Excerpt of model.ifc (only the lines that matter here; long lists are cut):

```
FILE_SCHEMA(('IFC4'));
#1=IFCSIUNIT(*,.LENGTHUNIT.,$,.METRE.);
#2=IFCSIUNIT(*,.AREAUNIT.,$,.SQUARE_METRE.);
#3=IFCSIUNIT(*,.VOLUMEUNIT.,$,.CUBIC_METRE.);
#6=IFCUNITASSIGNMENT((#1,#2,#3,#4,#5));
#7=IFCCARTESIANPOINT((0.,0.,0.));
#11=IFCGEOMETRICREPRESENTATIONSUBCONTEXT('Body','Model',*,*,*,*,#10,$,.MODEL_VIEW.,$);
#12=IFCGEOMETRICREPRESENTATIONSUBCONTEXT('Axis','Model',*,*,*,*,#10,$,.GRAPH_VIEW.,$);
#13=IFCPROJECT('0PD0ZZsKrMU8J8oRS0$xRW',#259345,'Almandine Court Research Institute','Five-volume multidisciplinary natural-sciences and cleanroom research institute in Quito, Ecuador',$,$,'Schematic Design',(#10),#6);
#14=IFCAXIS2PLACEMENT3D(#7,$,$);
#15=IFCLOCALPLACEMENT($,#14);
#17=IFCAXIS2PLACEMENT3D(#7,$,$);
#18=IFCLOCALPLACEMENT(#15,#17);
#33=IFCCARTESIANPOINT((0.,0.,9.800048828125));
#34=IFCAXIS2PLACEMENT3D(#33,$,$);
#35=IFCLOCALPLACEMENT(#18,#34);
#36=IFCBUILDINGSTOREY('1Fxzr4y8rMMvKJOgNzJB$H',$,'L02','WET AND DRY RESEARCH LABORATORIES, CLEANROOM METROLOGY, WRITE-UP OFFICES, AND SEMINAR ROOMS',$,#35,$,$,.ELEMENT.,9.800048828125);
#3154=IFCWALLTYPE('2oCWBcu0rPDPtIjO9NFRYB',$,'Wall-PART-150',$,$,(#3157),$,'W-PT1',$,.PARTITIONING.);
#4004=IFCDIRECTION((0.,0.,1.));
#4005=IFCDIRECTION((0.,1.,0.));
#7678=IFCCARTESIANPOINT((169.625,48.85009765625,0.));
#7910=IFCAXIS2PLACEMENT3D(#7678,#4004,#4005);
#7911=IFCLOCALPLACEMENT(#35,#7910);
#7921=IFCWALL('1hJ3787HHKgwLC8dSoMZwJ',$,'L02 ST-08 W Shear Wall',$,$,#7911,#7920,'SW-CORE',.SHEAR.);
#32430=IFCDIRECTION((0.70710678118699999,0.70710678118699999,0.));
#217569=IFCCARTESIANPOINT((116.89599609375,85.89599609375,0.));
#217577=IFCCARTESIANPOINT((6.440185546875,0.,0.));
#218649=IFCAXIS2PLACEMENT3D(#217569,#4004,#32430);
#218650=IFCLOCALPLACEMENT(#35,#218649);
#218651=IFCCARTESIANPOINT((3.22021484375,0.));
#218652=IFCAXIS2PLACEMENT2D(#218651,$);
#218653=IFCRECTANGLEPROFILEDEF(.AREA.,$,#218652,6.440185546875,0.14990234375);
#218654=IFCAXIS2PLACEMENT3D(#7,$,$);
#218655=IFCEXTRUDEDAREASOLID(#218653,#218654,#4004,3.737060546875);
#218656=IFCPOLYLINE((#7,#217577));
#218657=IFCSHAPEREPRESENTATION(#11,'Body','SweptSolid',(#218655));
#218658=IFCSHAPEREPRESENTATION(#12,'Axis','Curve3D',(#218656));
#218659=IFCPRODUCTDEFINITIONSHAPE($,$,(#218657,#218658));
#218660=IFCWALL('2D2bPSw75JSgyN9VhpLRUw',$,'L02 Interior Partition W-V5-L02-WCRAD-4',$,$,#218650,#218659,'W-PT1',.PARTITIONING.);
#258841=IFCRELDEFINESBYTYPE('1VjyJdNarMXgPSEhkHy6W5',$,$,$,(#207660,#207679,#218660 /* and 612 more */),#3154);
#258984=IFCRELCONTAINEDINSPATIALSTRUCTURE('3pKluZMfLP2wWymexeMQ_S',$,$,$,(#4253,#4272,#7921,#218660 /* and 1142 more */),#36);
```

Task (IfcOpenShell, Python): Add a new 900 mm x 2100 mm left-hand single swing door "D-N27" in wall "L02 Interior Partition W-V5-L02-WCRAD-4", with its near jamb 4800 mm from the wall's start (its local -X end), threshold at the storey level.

```python
import numpy as np
import ifcopenshell
import ifcopenshell.api.feature
import ifcopenshell.api.geometry
import ifcopenshell.api.root
import ifcopenshell.api.spatial
import ifcopenshell.geom
import ifcopenshell.util.element
import ifcopenshell.util.placement
import ifcopenshell.util.representation
import ifcopenshell.util.shape
import ifcopenshell.util.unit

model = ifcopenshell.open("model.ifc")
unit_scale = ifcopenshell.util.unit.calculate_unit_scale(model)
settings = ifcopenshell.geom.settings()


def volume(element):
    """Net volume in cubic metres, openings subtracted."""
    shape = ifcopenshell.geom.create_shape(settings, element)
    return ifcopenshell.util.shape.get_volume(shape.geometry)


wall = model.by_guid("2D2bPSw75JSgyN9VhpLRUw")
storey = ifcopenshell.util.element.get_container(wall, ifc_class="IfcBuildingStorey")
context = ifcopenshell.util.representation.get_context(model, "Model", "Body", "MODEL_VIEW")
before = volume(wall)

width, height, from_end, sill = 0.9, 2.1, 4.8, 0.0  # metres

# The wall runs along its own X axis, and the end named is its -X end.
wall_shape = ifcopenshell.geom.create_shape(settings, wall)
x, y, z = ifcopenshell.util.shape.get_vertices(wall_shape.geometry).T
start = x.min() + from_end
face, thickness = float(y.min()), float(y.max() - y.min())
wall_matrix = ifcopenshell.util.placement.get_local_placement(wall.ObjectPlacement)
level = ifcopenshell.util.placement.get_local_placement(storey.ObjectPlacement)[2, 3]


def in_wall(x, y):
    """Placement at x, y metres in the wall's axes, at sill height."""
    matrix = wall_matrix.copy()
    matrix[:, 3] = wall_matrix @ np.array([x / unit_scale, y / unit_scale, 0.0, 1.0])
    matrix[2, 3] = level + sill / unit_scale
    return matrix


# Opening: a box that overshoots both wall faces by 50 mm.
opening = ifcopenshell.api.root.create_entity(model, ifc_class="IfcOpeningElement", predefined_type="OPENING")
box = ifcopenshell.api.geometry.add_wall_representation(
    model, context=context, length=width, height=height, thickness=thickness + 0.1
)
ifcopenshell.api.geometry.assign_representation(model, product=opening, representation=box)
ifcopenshell.api.geometry.edit_object_placement(model, product=opening, matrix=in_wall(start, face - 0.05), is_si=False)
ifcopenshell.api.feature.add_feature(model, feature=opening, element=wall)

door = ifcopenshell.api.root.create_entity(model, ifc_class="IfcDoor", name="D-N27", predefined_type="DOOR")
door.OverallWidth, door.OverallHeight = width / unit_scale, height / unit_scale
door.OperationType = "SINGLE_SWING_LEFT"
body = ifcopenshell.api.geometry.add_door_representation(
    model,
    context=context,
    overall_width=door.OverallWidth,
    overall_height=door.OverallHeight,
    operation_type="SINGLE_SWING_LEFT",
    lining_properties={"LiningDepth": thickness / unit_scale, "ThresholdDepth": thickness / unit_scale},
)
ifcopenshell.api.geometry.assign_representation(model, product=door, representation=body)
ifcopenshell.api.spatial.assign_container(model, products=[door], relating_structure=storey)
ifcopenshell.api.feature.add_filling(model, opening=opening, element=door)

# The lining spans the wall, so the door starts at the wall face.
ifcopenshell.api.geometry.edit_object_placement(model, product=door, matrix=in_wall(start, face), is_si=False)

after = volume(wall)

print(f"wall volume {before:.3f} -> {after:.3f} m3")

model.write("model_rev.ifc")
```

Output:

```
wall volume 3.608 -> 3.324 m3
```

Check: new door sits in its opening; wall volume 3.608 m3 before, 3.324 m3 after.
